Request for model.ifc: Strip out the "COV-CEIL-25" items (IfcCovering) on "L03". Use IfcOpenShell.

First a look at what the model holds.

```python
import ifcopenshell
import ifcopenshell.util.element

model = ifcopenshell.open("model.ifc")
print(model.schema)
storey = next(s for s in model.by_type("IfcBuildingStorey") if s.Name == "L03")
coverings = [e for e in ifcopenshell.util.element.get_decomposition(storey) if e.is_a("IfcCovering")]
seen = {}
for e in coverings:
    element_type = ifcopenshell.util.element.get_type(e)
    name = element_type.Name if element_type not in (None, e) else None
    seen[name] = seen.get(name, 0) + 1
for name, count in sorted(seen.items(), key=str):
    print(count, "x", name)
```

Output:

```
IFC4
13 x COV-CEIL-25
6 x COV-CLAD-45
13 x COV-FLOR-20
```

```python
import ifcopenshell
import ifcopenshell.api.root
import ifcopenshell.util.element

model = ifcopenshell.open("model.ifc")

storey = next(s for s in model.by_type("IfcBuildingStorey") if s.Name == "L03")
coverings = [e for e in ifcopenshell.util.element.get_decomposition(storey) if e.is_a("IfcCovering")]
targets = [e for e in coverings if (t := ifcopenshell.util.element.get_type(e)) not in (None, e) and t.Name == "COV-CEIL-25"]

for e in targets:
    ifcopenshell.api.root.remove_product(model, product=e)
print(len(targets), "removed")

model.write("model_edited.ifc")
```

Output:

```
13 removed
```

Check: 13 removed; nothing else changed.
